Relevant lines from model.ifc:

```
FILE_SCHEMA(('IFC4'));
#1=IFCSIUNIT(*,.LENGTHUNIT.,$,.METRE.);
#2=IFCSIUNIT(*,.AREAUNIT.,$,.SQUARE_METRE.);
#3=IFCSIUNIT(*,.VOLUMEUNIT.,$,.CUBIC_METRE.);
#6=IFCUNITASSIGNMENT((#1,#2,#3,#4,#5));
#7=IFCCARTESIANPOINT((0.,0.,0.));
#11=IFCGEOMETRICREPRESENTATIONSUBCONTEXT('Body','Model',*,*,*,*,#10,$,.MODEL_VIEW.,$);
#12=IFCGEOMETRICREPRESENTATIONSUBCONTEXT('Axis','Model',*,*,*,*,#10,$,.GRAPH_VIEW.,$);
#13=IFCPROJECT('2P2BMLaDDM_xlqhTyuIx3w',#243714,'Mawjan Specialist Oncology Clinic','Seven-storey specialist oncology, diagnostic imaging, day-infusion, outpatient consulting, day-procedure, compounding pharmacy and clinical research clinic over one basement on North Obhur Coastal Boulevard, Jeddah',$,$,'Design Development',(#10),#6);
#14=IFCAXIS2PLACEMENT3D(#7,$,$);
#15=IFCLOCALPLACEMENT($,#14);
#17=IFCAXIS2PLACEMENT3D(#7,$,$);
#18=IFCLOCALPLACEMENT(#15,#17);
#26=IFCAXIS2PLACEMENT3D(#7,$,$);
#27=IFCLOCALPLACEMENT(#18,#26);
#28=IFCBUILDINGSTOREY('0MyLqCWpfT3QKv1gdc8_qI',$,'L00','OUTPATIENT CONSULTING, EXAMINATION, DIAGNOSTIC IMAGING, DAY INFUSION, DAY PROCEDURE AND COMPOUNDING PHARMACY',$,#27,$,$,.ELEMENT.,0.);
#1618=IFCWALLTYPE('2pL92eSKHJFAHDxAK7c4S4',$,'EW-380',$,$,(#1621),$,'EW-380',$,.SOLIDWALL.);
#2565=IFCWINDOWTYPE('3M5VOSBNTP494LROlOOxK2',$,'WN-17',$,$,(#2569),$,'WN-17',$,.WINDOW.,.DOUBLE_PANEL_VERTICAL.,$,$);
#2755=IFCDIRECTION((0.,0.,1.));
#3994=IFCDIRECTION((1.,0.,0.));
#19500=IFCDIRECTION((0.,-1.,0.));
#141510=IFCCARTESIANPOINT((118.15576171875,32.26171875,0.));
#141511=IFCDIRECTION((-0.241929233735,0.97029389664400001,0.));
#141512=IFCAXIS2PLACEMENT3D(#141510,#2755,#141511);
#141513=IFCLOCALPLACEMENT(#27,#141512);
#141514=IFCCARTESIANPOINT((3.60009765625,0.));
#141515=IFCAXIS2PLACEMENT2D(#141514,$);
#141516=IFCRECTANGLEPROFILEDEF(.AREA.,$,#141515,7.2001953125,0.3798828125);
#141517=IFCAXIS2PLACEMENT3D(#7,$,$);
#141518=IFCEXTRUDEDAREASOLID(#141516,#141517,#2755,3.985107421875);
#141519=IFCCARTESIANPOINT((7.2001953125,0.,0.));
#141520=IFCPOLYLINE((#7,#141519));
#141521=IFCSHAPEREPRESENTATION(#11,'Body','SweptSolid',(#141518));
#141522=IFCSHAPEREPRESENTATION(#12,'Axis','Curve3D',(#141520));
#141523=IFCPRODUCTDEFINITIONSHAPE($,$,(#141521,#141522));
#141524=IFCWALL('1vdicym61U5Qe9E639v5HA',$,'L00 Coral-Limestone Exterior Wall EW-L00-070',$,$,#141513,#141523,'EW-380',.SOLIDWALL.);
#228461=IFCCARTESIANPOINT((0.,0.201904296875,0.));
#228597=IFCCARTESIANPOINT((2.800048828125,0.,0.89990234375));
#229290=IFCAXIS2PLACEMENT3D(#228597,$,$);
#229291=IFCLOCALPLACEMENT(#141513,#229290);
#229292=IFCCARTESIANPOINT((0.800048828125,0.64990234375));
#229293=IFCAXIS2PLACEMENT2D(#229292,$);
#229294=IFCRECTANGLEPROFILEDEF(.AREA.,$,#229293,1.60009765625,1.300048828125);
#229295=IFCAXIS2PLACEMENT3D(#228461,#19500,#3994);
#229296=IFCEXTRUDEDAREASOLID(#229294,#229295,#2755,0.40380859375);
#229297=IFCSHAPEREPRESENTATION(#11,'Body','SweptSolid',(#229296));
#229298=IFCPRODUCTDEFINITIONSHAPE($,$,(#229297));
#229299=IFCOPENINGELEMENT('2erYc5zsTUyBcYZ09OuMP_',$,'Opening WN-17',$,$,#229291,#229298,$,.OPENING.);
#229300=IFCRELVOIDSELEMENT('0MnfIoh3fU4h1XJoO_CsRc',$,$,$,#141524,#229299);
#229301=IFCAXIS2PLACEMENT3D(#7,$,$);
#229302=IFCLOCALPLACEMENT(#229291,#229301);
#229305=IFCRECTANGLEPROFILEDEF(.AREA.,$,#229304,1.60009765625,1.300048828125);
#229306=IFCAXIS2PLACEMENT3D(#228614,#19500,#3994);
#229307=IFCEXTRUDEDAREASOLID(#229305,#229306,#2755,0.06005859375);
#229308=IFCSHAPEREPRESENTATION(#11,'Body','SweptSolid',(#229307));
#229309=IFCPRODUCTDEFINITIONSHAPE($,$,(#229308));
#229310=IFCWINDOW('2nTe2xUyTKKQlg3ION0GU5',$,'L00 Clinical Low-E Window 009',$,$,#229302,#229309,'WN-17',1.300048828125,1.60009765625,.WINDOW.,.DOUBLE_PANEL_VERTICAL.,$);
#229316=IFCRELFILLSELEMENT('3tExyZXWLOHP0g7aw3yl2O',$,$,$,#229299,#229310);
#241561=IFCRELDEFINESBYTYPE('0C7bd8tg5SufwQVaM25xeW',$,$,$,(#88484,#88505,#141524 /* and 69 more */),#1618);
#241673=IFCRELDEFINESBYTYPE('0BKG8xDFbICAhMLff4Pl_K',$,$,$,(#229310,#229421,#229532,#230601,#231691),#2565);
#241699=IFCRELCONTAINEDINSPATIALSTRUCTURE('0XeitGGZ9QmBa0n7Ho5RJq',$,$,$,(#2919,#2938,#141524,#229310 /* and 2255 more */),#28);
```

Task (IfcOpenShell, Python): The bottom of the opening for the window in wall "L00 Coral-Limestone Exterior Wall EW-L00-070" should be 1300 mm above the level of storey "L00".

```python
import numpy as np
import ifcopenshell
import ifcopenshell.api.geometry
import ifcopenshell.geom
import ifcopenshell.util.element
import ifcopenshell.util.placement
import ifcopenshell.util.shape
import ifcopenshell.util.unit

model = ifcopenshell.open("model.ifc")
unit_scale = ifcopenshell.util.unit.calculate_unit_scale(model)

window = model.by_guid("2nTe2xUyTKKQlg3ION0GU5")
opening = window.FillsVoids[0].RelatingOpeningElement
storey = ifcopenshell.util.element.get_container(window, ifc_class="IfcBuildingStorey")
level = ifcopenshell.util.placement.get_local_placement(storey.ObjectPlacement)[2, 3]

# The opening's origin need not be at the sill, so measure its lowest point.
shape = ifcopenshell.geom.create_shape(ifcopenshell.geom.settings(), opening)
bottom = ifcopenshell.util.shape.get_shape_bottom_elevation(shape, shape.geometry) / unit_scale
dz = level + 1.3 / unit_scale - bottom

shift = np.array([0.0, 0.0, dz])
# The window is placed relative to its opening, so it follows when the opening moves.
matrix = ifcopenshell.util.placement.get_local_placement(opening.ObjectPlacement)
matrix[:3, 3] += shift
ifcopenshell.api.geometry.edit_object_placement(
    model, product=opening, matrix=matrix, is_si=False, should_transform_children=True
)

print(f"moved by {dz * unit_scale:+.3f} m")

model.write("model_edited.ifc")
```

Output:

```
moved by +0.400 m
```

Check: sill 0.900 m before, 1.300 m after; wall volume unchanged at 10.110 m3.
